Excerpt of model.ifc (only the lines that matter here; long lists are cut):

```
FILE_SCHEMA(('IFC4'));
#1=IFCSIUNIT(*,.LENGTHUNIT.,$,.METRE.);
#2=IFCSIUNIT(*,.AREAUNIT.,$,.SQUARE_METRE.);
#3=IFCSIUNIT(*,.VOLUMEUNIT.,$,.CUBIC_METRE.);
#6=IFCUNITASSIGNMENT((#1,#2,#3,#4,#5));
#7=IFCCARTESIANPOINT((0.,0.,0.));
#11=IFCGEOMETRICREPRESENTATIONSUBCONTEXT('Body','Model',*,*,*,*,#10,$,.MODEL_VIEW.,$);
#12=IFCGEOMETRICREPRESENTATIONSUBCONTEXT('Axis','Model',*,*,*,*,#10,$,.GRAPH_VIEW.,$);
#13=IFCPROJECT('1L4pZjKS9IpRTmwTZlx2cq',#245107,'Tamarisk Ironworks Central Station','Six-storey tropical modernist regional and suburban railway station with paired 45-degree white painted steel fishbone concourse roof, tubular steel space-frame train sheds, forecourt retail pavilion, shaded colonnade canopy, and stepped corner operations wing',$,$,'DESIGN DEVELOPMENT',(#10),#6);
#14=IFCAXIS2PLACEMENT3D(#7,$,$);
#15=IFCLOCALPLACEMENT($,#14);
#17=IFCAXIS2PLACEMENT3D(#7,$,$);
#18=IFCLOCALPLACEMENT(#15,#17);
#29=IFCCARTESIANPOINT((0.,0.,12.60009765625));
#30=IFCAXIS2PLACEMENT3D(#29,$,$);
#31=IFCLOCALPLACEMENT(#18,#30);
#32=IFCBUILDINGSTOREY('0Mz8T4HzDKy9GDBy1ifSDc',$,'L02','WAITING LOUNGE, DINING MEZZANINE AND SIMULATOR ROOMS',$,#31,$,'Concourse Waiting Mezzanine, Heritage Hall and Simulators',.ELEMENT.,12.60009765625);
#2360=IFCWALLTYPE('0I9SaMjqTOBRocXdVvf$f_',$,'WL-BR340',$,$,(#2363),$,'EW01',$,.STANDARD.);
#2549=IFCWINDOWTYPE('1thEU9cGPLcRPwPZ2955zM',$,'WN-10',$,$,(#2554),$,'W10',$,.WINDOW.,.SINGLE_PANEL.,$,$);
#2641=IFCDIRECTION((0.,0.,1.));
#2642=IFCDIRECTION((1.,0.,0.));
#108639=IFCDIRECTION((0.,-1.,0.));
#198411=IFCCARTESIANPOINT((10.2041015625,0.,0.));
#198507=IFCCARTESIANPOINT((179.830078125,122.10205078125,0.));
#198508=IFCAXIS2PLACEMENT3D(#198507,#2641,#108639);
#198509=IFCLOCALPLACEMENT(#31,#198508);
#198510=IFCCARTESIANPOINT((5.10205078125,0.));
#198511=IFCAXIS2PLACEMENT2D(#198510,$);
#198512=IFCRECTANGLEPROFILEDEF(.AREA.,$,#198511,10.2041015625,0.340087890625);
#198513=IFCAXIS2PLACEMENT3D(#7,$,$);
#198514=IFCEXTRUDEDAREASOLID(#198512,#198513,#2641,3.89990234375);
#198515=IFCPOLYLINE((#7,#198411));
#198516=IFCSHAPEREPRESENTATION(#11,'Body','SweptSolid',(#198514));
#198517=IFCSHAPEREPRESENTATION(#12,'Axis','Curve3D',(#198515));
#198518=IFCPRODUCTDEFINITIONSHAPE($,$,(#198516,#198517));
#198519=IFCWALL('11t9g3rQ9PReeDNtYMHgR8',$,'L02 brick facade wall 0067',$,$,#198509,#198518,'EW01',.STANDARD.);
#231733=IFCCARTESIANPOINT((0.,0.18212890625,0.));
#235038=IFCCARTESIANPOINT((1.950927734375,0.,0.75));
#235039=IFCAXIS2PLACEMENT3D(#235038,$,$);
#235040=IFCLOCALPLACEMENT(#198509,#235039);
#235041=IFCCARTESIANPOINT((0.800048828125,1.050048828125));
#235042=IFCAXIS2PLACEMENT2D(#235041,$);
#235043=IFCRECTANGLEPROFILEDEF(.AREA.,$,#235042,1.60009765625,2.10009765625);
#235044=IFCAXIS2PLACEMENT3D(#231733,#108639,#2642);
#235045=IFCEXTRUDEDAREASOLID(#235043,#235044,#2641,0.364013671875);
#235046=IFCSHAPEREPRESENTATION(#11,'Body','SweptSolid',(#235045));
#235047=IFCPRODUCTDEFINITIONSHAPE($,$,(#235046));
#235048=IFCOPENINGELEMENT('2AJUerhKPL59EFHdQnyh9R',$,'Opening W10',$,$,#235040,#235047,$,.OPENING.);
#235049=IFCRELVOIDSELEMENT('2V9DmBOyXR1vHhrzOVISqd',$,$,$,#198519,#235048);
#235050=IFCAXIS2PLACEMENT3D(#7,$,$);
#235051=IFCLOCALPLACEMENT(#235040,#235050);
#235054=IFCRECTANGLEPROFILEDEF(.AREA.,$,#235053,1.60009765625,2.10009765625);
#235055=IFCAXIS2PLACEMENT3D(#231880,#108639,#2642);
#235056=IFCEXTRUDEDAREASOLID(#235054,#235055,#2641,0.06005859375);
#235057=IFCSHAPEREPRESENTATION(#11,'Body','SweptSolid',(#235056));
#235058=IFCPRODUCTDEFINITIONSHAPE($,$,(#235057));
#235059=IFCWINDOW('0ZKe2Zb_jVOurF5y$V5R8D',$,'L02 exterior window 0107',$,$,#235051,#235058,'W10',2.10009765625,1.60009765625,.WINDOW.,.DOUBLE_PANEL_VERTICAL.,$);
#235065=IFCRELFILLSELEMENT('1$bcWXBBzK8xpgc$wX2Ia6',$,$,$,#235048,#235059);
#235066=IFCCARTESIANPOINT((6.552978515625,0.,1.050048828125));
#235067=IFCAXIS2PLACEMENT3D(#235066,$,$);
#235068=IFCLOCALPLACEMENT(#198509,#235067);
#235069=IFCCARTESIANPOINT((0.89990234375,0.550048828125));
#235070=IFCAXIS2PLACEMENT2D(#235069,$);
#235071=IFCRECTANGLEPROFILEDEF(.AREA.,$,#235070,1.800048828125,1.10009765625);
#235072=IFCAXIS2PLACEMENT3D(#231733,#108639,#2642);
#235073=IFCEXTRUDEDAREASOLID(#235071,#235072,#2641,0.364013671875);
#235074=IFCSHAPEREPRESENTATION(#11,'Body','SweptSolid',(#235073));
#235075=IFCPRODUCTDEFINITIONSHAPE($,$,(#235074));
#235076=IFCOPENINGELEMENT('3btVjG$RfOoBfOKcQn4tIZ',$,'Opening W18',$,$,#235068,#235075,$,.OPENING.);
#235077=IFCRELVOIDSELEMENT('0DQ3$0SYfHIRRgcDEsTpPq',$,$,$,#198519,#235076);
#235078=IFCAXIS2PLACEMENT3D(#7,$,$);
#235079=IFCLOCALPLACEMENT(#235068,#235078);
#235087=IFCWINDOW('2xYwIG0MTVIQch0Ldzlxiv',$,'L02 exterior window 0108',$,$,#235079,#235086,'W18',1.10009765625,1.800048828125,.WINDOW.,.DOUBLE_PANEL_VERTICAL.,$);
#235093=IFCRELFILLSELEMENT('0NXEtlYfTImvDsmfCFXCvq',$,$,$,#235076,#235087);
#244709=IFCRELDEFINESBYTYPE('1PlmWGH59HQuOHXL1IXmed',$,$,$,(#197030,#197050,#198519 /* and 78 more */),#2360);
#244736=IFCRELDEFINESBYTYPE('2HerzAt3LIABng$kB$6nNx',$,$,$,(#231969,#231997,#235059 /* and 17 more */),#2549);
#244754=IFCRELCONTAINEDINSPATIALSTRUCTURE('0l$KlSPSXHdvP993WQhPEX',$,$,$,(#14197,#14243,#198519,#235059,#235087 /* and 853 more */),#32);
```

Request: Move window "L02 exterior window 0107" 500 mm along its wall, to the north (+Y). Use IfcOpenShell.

```python
import ifcopenshell
import ifcopenshell.api.geometry
import ifcopenshell.util.placement
import ifcopenshell.util.unit

model = ifcopenshell.open("model.ifc")
unit_scale = ifcopenshell.util.unit.calculate_unit_scale(model)

window = model.by_guid("0ZKe2Zb_jVOurF5y$V5R8D")
opening = window.FillsVoids[0].RelatingOpeningElement
wall = opening.VoidsElements[0].RelatingBuildingElement

wall_matrix = ifcopenshell.util.placement.get_local_placement(wall.ObjectPlacement)
shift = wall_matrix[:3, 0] * -0.5 / unit_scale
before = ifcopenshell.util.placement.get_local_placement(window.ObjectPlacement)[:3, 3].copy()

# The window is placed relative to its opening, so it follows when the opening moves.
matrix = ifcopenshell.util.placement.get_local_placement(opening.ObjectPlacement)
matrix[:3, 3] += shift
ifcopenshell.api.geometry.edit_object_placement(
    model, product=opening, matrix=matrix, is_si=False, should_transform_children=True
)

after = ifcopenshell.util.placement.get_local_placement(window.ObjectPlacement)[:3, 3]
print("window moved by", (after - before).round(3) + 0.0)

model.write("model_rev.ifc")
```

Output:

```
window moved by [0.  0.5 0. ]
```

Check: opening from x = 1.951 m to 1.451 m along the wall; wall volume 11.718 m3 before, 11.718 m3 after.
